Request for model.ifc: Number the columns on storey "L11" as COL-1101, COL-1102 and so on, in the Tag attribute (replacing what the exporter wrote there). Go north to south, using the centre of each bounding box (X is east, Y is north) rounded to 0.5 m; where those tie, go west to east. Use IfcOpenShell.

First a look at what the model holds.

```python
import ifcopenshell
import ifcopenshell.util.element
import ifcopenshell.util.placement

model = ifcopenshell.open("model.ifc")
print(model.schema)
storey = next(s for s in model.by_type("IfcBuildingStorey") if s.Name == "L11")
columns = [e for e in ifcopenshell.util.element.get_decomposition(storey) if e.is_a("IfcColumn")]
for e in sorted(columns, key=lambda e: e.id()):
    origin = ifcopenshell.util.placement.get_local_placement(e.ObjectPlacement)[:3, 3]
    print(e.id(), e.Tag, e.Name, origin.round(2) + 0.0, sep=" | ")
```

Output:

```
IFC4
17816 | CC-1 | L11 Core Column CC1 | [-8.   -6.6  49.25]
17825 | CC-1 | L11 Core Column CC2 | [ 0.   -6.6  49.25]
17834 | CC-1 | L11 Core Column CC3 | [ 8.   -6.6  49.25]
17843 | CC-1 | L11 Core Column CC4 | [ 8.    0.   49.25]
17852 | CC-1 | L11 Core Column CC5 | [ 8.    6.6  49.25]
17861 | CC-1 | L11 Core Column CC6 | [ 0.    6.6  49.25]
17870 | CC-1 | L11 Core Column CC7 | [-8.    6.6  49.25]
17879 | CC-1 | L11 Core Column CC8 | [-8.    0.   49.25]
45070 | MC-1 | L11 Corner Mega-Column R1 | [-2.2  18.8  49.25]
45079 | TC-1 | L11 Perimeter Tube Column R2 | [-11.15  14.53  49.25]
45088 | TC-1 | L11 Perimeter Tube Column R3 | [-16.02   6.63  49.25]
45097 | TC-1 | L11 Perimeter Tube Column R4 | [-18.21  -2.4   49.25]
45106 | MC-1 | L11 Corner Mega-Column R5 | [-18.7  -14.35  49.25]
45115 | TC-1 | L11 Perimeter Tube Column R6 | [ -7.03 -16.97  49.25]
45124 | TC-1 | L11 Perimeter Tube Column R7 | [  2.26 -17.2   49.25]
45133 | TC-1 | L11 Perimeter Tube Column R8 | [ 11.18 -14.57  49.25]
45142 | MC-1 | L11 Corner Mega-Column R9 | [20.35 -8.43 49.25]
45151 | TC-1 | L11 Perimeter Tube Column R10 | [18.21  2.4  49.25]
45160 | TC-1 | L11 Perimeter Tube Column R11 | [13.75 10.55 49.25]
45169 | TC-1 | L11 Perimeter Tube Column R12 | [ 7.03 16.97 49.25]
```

```python
import ifcopenshell
import ifcopenshell.geom
import ifcopenshell.util.element
import ifcopenshell.util.shape

model = ifcopenshell.open("model.ifc")
settings = ifcopenshell.geom.settings()
settings.set("use-world-coords", True)


def centre(element):
    shape = ifcopenshell.geom.create_shape(settings, element)
    return ifcopenshell.util.shape.get_bbox_centroid(shape.geometry)


storey = next(s for s in model.by_type("IfcBuildingStorey") if s.Name == "L11")
columns = [e for e in ifcopenshell.util.element.get_decomposition(storey) if e.is_a("IfcColumn")]

# Insertion points can sit at a corner or the storey origin, so sort by the geometry (in metres).
centres = {e: centre(e) for e in columns}
columns.sort(key=lambda e: (-round(centres[e][1] / 0.5), centres[e][0]))

for i, e in enumerate(columns, start=1):
    number = f"COL-11{i:02d}"
    e.Tag = number
    print(e.id(), number)

model.write("model_v2.ifc")
```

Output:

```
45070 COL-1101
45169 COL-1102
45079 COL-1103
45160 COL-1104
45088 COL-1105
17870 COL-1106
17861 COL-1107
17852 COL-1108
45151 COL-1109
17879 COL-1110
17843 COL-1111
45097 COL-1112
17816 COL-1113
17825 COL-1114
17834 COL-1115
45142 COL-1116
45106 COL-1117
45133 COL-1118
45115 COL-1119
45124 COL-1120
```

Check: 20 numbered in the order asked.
